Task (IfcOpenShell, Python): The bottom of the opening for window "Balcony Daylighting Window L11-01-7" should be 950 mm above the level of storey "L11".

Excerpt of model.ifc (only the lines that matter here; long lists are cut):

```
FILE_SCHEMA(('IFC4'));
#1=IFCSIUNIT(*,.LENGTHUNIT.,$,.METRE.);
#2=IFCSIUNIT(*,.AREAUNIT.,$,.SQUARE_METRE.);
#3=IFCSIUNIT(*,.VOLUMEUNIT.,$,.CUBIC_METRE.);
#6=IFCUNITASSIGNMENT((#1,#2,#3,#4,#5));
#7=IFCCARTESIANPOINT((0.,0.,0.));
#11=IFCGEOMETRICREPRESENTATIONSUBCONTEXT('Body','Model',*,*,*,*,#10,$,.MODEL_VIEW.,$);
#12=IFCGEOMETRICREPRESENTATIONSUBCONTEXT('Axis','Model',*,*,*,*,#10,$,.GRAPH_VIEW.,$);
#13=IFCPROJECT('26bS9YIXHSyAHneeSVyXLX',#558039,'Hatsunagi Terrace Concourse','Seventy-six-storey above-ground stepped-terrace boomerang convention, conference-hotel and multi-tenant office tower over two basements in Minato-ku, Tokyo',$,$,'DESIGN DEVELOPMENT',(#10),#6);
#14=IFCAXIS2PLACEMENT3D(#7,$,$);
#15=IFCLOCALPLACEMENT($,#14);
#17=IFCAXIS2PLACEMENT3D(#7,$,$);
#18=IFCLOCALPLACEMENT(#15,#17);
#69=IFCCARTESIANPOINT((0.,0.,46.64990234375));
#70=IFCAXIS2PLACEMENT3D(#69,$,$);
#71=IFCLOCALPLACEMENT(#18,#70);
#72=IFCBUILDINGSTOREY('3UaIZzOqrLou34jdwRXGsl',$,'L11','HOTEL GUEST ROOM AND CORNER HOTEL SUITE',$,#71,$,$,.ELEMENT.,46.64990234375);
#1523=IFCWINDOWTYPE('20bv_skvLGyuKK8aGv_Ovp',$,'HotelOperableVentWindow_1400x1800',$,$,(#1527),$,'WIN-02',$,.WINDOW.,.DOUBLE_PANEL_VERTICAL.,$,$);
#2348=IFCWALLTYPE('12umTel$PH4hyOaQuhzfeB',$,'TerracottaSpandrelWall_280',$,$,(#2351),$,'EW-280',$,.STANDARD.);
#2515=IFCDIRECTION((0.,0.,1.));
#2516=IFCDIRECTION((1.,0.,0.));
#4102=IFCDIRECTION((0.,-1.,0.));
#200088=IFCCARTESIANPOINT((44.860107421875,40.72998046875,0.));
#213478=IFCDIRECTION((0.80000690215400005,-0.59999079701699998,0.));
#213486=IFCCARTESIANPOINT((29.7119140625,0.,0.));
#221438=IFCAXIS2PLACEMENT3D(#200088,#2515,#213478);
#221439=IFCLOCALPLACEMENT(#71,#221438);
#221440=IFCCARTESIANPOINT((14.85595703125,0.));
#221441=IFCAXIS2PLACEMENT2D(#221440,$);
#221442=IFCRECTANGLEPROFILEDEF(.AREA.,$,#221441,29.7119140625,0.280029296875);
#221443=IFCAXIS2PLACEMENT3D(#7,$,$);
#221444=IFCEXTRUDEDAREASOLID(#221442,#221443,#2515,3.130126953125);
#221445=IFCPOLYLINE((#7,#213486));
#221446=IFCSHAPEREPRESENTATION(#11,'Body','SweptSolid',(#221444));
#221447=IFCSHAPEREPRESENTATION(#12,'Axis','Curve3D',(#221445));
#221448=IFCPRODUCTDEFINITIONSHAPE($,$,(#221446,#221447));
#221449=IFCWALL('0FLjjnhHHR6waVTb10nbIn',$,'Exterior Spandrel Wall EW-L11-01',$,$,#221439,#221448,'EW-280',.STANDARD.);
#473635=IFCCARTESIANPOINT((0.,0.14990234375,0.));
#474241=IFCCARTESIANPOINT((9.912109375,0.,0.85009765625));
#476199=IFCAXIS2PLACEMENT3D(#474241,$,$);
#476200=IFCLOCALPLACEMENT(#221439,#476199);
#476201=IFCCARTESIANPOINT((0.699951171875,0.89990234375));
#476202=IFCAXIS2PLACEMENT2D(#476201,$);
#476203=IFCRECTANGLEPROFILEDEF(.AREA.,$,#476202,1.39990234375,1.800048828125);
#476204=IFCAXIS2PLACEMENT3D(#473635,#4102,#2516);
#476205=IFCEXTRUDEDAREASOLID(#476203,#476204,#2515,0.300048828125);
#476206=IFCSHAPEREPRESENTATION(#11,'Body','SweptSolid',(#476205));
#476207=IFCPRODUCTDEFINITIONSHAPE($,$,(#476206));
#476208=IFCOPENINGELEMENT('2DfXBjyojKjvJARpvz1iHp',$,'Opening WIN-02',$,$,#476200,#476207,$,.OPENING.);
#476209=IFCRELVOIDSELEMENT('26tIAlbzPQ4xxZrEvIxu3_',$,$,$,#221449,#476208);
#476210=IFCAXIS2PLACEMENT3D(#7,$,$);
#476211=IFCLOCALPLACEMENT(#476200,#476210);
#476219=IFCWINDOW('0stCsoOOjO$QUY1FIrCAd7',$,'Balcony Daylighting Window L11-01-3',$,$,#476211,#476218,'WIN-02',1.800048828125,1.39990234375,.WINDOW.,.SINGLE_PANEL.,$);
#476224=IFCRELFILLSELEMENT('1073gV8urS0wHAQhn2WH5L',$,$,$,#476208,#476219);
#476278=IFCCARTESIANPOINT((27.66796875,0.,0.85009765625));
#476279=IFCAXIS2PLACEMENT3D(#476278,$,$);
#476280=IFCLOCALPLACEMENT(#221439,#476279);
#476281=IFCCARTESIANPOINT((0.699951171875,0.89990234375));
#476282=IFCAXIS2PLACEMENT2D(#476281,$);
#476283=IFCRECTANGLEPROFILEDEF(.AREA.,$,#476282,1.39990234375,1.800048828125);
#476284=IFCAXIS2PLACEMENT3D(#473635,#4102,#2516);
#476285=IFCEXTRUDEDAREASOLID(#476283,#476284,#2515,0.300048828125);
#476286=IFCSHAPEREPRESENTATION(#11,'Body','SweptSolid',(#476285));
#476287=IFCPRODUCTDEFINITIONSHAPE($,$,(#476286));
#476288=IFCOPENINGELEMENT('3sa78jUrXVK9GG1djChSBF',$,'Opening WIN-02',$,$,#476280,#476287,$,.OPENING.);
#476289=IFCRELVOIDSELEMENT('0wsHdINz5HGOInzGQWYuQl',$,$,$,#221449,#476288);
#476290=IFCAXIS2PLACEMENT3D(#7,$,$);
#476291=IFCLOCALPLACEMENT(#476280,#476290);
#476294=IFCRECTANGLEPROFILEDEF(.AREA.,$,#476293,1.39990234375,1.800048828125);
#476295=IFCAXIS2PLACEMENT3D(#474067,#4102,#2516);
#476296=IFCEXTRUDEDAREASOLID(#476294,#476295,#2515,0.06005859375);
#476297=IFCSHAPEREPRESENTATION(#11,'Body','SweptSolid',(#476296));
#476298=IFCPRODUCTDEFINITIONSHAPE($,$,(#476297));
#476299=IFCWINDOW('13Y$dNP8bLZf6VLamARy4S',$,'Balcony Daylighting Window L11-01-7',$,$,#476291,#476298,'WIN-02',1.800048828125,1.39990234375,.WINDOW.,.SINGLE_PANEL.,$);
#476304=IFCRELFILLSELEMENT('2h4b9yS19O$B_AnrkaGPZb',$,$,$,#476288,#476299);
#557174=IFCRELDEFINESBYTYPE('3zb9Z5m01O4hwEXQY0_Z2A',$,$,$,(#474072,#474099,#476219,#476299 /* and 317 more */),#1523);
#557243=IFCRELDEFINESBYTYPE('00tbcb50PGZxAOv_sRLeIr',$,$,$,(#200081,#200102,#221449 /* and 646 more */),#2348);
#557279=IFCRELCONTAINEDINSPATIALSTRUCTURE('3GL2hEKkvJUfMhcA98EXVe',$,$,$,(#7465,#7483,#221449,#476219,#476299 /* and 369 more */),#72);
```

```python
import numpy as np
import ifcopenshell
import ifcopenshell.api.geometry
import ifcopenshell.geom
import ifcopenshell.util.element
import ifcopenshell.util.placement
import ifcopenshell.util.shape
import ifcopenshell.util.unit

model = ifcopenshell.open("model.ifc")
unit_scale = ifcopenshell.util.unit.calculate_unit_scale(model)

window = model.by_id(476299)
opening = window.FillsVoids[0].RelatingOpeningElement
storey = ifcopenshell.util.element.get_container(window, ifc_class="IfcBuildingStorey")
level = ifcopenshell.util.placement.get_local_placement(storey.ObjectPlacement)[2, 3]

# The opening's origin need not be at the sill, so measure its lowest point.
shape = ifcopenshell.geom.create_shape(ifcopenshell.geom.settings(), opening)
bottom = ifcopenshell.util.shape.get_shape_bottom_elevation(shape, shape.geometry) / unit_scale
dz = level + 0.95 - bottom

shift = np.array([0.0, 0.0, dz])
# The window is placed relative to its opening, so it follows when the opening moves.
matrix = ifcopenshell.util.placement.get_local_placement(opening.ObjectPlacement)
matrix[:3, 3] += shift
ifcopenshell.api.geometry.edit_object_placement(
    model, product=opening, matrix=matrix, is_si=False, should_transform_children=True
)

print(f"moved by {dz * unit_scale:+.3f} m")

model.write("model_rev.ifc")
```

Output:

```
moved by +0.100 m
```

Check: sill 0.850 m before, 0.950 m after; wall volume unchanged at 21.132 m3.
